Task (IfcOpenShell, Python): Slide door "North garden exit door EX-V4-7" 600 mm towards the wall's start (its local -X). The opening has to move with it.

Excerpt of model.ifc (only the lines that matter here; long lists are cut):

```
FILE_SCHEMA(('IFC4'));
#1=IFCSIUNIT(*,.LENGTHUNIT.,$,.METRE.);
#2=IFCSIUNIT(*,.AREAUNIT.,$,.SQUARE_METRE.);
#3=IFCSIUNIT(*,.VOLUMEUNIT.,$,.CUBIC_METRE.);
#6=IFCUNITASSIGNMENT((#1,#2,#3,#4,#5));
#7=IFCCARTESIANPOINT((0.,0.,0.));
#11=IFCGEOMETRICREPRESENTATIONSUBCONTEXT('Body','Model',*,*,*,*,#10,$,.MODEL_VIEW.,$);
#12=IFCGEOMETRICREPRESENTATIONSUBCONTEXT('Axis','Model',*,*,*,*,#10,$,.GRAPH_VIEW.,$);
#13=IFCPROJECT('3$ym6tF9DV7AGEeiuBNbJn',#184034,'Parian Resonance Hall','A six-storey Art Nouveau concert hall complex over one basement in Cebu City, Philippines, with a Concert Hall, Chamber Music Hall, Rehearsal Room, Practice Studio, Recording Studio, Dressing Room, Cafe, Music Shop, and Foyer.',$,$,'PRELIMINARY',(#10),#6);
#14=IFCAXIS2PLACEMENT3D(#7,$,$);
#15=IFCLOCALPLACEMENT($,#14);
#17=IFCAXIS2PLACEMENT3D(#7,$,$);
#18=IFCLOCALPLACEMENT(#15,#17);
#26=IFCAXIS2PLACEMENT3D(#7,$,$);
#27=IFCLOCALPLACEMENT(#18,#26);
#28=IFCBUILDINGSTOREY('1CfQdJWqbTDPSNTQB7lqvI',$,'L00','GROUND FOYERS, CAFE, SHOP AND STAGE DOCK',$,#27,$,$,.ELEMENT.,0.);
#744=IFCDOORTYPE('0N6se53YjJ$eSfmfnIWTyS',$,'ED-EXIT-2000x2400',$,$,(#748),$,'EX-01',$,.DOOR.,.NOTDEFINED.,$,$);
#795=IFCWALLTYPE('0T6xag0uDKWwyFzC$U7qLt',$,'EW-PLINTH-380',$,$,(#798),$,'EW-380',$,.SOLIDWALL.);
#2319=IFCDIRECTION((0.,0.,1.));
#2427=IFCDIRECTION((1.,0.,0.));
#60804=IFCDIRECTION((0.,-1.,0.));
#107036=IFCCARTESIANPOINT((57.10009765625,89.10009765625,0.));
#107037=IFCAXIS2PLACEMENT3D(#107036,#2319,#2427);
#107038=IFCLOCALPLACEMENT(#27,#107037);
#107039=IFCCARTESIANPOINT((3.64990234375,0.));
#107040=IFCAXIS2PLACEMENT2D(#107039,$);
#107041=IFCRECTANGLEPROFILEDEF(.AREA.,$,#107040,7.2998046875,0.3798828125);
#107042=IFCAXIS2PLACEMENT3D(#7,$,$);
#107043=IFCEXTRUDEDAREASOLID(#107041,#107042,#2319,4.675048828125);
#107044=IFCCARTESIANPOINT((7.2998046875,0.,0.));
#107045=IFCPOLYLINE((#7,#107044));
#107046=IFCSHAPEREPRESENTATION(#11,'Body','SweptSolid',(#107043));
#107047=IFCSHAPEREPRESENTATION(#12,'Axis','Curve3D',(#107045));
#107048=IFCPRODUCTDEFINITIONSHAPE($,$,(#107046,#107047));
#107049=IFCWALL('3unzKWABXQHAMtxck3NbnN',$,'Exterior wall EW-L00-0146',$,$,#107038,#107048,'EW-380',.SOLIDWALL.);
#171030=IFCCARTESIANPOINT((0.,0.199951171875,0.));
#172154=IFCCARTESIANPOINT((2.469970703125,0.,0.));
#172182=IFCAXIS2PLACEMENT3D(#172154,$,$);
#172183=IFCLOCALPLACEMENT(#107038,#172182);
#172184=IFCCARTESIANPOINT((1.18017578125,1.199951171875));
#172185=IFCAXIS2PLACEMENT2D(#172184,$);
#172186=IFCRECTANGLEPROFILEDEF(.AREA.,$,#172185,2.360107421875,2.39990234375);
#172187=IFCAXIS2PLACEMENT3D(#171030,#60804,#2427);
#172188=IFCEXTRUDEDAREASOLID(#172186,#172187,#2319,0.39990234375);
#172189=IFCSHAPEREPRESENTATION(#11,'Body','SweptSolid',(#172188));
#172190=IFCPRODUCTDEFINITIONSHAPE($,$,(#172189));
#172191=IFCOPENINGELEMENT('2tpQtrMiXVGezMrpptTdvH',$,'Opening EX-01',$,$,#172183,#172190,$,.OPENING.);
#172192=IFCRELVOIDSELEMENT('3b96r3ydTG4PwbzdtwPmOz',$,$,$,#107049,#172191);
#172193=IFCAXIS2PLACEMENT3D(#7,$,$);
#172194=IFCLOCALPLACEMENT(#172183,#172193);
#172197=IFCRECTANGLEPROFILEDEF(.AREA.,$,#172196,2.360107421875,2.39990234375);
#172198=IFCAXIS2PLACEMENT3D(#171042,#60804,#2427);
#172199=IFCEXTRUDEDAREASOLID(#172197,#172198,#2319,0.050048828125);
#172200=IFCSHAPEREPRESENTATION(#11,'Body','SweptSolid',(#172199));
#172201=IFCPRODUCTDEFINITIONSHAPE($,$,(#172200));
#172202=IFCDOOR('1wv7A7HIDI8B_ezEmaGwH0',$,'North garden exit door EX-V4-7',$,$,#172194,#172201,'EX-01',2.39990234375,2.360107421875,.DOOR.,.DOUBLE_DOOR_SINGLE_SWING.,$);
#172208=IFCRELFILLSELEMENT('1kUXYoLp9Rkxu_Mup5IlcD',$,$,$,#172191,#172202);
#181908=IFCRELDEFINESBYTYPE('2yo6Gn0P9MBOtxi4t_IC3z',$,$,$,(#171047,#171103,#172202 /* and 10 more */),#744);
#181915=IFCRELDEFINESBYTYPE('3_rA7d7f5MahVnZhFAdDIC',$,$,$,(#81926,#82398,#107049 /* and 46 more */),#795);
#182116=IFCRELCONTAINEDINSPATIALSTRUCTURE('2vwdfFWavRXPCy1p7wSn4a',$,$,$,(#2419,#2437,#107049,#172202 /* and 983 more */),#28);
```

```python
import ifcopenshell
import ifcopenshell.api.geometry
import ifcopenshell.util.placement

model = ifcopenshell.open("model.ifc")

door = model.by_guid("1wv7A7HIDI8B_ezEmaGwH0")
opening = door.FillsVoids[0].RelatingOpeningElement
wall = opening.VoidsElements[0].RelatingBuildingElement

wall_matrix = ifcopenshell.util.placement.get_local_placement(wall.ObjectPlacement)
shift = wall_matrix[:3, 0] * -0.6
before = ifcopenshell.util.placement.get_local_placement(door.ObjectPlacement)[:3, 3].copy()

# The door is placed relative to its opening, so it follows when the opening moves.
matrix = ifcopenshell.util.placement.get_local_placement(opening.ObjectPlacement)
matrix[:3, 3] += shift
ifcopenshell.api.geometry.edit_object_placement(
    model, product=opening, matrix=matrix, is_si=False, should_transform_children=True
)

after = ifcopenshell.util.placement.get_local_placement(door.ObjectPlacement)[:3, 3]
print("door moved by", (after - before).round(3) + 0.0)

model.write("model_updated.ifc")
```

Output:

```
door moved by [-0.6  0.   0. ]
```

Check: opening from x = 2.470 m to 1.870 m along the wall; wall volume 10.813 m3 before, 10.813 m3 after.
